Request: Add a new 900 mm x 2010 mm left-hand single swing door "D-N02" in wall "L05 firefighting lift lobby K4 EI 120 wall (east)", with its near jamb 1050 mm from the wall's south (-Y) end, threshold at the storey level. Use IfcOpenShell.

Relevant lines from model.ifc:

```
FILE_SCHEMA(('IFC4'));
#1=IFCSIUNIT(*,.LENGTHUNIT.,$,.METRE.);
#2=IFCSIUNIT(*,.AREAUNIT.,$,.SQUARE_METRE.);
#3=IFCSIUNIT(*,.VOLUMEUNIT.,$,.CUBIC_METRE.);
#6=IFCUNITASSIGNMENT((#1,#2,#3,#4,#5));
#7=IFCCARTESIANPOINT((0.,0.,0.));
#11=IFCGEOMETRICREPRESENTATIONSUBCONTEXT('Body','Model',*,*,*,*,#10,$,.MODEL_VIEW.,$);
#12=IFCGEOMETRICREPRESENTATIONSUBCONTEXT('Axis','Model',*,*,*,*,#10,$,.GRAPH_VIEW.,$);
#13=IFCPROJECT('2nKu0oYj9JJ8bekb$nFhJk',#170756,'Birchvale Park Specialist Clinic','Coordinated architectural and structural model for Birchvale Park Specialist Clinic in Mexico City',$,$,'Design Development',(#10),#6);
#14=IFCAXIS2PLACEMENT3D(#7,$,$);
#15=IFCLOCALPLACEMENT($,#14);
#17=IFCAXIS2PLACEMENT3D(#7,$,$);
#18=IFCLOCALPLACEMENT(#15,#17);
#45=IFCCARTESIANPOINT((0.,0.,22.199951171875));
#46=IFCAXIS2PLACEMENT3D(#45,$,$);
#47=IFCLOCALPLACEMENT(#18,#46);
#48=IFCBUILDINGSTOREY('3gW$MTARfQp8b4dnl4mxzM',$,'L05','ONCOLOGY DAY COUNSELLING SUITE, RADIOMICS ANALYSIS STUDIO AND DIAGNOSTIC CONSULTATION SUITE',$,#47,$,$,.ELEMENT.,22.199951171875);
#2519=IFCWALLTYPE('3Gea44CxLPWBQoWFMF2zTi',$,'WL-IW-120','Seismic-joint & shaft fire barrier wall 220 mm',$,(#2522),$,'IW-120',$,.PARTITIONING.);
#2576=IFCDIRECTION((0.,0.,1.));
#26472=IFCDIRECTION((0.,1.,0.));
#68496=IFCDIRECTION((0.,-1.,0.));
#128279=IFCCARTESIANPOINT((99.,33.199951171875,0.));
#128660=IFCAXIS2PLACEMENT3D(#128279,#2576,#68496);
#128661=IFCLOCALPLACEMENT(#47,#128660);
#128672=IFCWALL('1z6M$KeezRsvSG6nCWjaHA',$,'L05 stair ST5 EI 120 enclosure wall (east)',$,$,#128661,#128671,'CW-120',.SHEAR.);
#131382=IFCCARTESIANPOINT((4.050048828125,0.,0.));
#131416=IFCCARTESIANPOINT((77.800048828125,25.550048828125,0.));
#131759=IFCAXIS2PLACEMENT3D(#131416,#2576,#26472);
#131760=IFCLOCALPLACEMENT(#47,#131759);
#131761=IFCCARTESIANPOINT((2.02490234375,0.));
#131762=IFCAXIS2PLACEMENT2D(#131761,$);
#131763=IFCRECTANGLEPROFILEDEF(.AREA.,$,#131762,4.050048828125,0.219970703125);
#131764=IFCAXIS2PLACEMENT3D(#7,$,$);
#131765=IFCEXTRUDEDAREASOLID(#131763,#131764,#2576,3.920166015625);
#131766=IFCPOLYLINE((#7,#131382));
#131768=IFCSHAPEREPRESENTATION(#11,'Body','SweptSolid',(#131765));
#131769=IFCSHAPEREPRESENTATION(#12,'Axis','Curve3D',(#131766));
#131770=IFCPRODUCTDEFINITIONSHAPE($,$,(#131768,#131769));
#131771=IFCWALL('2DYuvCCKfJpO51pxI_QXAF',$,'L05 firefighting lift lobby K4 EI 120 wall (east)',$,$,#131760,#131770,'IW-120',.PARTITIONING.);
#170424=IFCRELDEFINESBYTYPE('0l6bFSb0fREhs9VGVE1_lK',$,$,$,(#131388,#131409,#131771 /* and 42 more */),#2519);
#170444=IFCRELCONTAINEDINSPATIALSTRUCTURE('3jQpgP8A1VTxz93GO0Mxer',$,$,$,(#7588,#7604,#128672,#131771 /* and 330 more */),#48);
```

```python
import numpy as np
import ifcopenshell
import ifcopenshell.api.feature
import ifcopenshell.api.geometry
import ifcopenshell.api.root
import ifcopenshell.api.spatial
import ifcopenshell.geom
import ifcopenshell.util.element
import ifcopenshell.util.placement
import ifcopenshell.util.representation
import ifcopenshell.util.shape
import ifcopenshell.util.unit

model = ifcopenshell.open("model.ifc")
unit_scale = ifcopenshell.util.unit.calculate_unit_scale(model)
settings = ifcopenshell.geom.settings()


def volume(element):
    """Net volume in cubic metres, openings subtracted."""
    shape = ifcopenshell.geom.create_shape(settings, element)
    return ifcopenshell.util.shape.get_volume(shape.geometry)


wall = model.by_guid("2DYuvCCKfJpO51pxI_QXAF")
storey = ifcopenshell.util.element.get_container(wall, ifc_class="IfcBuildingStorey")
context = ifcopenshell.util.representation.get_context(model, "Model", "Body", "MODEL_VIEW")
before = volume(wall)

width, height, from_end, sill = 0.9, 2.01, 1.05, 0.0  # metres

# The wall runs along its own X axis, and the end named is its -X end.
wall_shape = ifcopenshell.geom.create_shape(settings, wall)
x, y, z = ifcopenshell.util.shape.get_vertices(wall_shape.geometry).T
start = x.min() + from_end
face, thickness = float(y.min()), float(y.max() - y.min())
wall_matrix = ifcopenshell.util.placement.get_local_placement(wall.ObjectPlacement)
level = ifcopenshell.util.placement.get_local_placement(storey.ObjectPlacement)[2, 3]


def in_wall(x, y):
    """Placement at x, y metres in the wall's axes, at sill height."""
    matrix = wall_matrix.copy()
    matrix[:, 3] = wall_matrix @ np.array([x / unit_scale, y / unit_scale, 0.0, 1.0])
    matrix[2, 3] = level + sill / unit_scale
    return matrix


# Opening: a box that overshoots both wall faces by 50 mm.
opening = ifcopenshell.api.root.create_entity(model, ifc_class="IfcOpeningElement", predefined_type="OPENING")
box = ifcopenshell.api.geometry.add_wall_representation(
    model, context=context, length=width, height=height, thickness=thickness + 0.1
)
ifcopenshell.api.geometry.assign_representation(model, product=opening, representation=box)
ifcopenshell.api.geometry.edit_object_placement(model, product=opening, matrix=in_wall(start, face - 0.05), is_si=False)
ifcopenshell.api.feature.add_feature(model, feature=opening, element=wall)

door = ifcopenshell.api.root.create_entity(model, ifc_class="IfcDoor", name="D-N02", predefined_type="DOOR")
door.OverallWidth, door.OverallHeight = width / unit_scale, height / unit_scale
door.OperationType = "SINGLE_SWING_LEFT"
body = ifcopenshell.api.geometry.add_door_representation(
    model,
    context=context,
    overall_width=door.OverallWidth,
    overall_height=door.OverallHeight,
    operation_type="SINGLE_SWING_LEFT",
    lining_properties={"LiningDepth": thickness / unit_scale, "ThresholdDepth": thickness / unit_scale},
)
ifcopenshell.api.geometry.assign_representation(model, product=door, representation=body)
ifcopenshell.api.spatial.assign_container(model, products=[door], relating_structure=storey)
ifcopenshell.api.feature.add_filling(model, opening=opening, element=door)

# The lining spans the wall, so the door starts at the wall face.
ifcopenshell.api.geometry.edit_object_placement(model, product=door, matrix=in_wall(start, face), is_si=False)

after = volume(wall)

print(f"wall volume {before:.3f} -> {after:.3f} m3")

model.write("model_v2.ifc")
```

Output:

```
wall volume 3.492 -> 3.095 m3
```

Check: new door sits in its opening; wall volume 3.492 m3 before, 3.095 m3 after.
